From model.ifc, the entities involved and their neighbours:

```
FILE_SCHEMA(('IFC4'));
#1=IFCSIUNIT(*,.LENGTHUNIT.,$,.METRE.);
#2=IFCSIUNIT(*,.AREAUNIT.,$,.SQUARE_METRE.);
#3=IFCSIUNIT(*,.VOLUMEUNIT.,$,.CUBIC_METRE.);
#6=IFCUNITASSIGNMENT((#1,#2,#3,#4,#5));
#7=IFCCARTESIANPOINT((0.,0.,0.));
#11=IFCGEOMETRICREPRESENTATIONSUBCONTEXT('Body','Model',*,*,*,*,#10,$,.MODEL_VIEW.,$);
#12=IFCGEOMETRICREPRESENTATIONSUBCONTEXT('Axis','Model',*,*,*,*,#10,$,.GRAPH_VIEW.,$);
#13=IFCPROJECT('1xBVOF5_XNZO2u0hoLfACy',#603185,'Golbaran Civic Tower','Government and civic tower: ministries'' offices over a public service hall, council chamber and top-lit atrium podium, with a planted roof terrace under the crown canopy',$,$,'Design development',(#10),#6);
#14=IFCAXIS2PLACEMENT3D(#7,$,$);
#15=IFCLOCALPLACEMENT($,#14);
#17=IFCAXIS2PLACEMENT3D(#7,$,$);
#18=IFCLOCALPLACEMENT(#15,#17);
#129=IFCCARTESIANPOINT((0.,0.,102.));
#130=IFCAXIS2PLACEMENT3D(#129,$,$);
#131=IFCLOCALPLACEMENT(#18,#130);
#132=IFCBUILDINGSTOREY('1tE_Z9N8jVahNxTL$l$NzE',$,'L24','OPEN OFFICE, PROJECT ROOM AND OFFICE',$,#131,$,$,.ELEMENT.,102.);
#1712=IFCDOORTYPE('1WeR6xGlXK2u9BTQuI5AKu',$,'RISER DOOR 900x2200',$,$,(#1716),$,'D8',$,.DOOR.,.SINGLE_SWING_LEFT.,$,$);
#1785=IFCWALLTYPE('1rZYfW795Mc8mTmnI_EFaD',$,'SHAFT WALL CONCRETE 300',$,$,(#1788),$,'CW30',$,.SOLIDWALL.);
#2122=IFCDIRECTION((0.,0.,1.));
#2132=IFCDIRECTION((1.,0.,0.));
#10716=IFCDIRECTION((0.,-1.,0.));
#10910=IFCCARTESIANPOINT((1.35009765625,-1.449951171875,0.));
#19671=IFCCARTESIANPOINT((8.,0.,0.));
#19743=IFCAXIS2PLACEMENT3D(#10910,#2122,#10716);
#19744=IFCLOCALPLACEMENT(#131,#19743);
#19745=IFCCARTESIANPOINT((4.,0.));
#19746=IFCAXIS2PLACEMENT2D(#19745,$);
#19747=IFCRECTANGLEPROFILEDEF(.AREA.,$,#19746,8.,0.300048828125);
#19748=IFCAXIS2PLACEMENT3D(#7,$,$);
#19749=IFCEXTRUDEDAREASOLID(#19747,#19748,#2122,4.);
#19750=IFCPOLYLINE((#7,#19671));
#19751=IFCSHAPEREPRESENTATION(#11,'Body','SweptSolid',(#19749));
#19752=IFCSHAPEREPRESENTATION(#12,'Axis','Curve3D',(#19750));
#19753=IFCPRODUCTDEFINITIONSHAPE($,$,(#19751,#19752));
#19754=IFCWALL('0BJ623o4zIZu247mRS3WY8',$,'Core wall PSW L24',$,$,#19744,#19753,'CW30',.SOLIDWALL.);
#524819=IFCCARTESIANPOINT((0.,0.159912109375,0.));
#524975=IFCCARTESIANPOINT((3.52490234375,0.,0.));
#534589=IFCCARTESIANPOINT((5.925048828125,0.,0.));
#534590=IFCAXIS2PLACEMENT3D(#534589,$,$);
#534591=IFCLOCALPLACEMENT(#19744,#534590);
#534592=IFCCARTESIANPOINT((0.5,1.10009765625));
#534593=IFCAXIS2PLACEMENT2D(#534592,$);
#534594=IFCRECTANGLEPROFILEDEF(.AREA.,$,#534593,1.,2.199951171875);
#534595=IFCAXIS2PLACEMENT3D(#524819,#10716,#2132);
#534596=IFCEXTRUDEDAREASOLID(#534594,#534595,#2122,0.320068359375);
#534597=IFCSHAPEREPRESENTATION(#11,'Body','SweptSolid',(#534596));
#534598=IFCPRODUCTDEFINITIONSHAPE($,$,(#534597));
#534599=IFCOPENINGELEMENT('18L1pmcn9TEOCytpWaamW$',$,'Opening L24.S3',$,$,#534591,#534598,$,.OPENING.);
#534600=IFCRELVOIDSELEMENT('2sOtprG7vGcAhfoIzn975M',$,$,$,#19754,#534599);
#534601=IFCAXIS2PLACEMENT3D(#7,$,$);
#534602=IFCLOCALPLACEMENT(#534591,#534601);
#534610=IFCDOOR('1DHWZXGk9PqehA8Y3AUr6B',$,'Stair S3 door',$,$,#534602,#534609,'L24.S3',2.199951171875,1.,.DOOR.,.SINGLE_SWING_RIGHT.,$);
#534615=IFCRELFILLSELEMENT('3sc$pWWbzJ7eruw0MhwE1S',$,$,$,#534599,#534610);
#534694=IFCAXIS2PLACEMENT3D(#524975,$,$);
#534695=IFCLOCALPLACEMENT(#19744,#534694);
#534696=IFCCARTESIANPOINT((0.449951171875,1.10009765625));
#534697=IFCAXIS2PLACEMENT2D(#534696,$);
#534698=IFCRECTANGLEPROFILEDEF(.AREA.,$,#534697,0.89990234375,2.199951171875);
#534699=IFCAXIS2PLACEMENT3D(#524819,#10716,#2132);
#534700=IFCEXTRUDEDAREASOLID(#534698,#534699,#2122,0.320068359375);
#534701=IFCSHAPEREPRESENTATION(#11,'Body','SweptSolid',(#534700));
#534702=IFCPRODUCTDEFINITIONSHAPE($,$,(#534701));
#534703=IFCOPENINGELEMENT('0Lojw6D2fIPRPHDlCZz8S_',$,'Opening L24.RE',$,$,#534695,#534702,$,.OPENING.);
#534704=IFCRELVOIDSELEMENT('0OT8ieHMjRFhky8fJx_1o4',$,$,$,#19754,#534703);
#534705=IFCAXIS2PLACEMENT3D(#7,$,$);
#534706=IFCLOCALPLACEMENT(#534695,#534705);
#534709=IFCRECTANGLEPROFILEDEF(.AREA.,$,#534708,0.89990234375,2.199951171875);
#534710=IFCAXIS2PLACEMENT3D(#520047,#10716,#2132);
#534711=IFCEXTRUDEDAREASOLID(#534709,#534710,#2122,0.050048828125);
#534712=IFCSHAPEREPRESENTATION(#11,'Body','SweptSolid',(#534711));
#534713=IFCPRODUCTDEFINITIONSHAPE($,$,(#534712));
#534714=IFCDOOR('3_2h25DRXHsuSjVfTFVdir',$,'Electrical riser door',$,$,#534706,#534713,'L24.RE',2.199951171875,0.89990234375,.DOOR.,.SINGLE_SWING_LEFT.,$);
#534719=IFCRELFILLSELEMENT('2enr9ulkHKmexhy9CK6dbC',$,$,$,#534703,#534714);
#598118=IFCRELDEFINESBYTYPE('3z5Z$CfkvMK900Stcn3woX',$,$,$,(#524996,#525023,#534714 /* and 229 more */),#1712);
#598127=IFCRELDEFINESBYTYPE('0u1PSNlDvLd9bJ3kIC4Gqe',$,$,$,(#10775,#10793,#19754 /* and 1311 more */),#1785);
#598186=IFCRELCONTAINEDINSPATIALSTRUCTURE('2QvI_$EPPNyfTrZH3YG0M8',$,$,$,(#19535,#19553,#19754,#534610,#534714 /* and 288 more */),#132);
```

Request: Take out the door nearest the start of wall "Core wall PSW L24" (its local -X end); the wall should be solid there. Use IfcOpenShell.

```python
import ifcopenshell
import ifcopenshell.api.feature
import ifcopenshell.api.root
import ifcopenshell.geom
import ifcopenshell.util.shape

model = ifcopenshell.open("model.ifc")
settings = ifcopenshell.geom.settings()


def volume(element):
    """Net volume in cubic metres, openings subtracted."""
    shape = ifcopenshell.geom.create_shape(settings, element)
    return ifcopenshell.util.shape.get_volume(shape.geometry)


door = model.by_id(534714)
opening = door.FillsVoids[0].RelatingOpeningElement
wall = opening.VoidsElements[0].RelatingBuildingElement
before = volume(wall)

ifcopenshell.api.root.remove_product(model, product=door)
ifcopenshell.api.feature.remove_feature(model, feature=opening)

after = volume(wall)

print(f"wall volume {before:.3f} -> {after:.3f} m3")

model.write("model_edited.ifc")
```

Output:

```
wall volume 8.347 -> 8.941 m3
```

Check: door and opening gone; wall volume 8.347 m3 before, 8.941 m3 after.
